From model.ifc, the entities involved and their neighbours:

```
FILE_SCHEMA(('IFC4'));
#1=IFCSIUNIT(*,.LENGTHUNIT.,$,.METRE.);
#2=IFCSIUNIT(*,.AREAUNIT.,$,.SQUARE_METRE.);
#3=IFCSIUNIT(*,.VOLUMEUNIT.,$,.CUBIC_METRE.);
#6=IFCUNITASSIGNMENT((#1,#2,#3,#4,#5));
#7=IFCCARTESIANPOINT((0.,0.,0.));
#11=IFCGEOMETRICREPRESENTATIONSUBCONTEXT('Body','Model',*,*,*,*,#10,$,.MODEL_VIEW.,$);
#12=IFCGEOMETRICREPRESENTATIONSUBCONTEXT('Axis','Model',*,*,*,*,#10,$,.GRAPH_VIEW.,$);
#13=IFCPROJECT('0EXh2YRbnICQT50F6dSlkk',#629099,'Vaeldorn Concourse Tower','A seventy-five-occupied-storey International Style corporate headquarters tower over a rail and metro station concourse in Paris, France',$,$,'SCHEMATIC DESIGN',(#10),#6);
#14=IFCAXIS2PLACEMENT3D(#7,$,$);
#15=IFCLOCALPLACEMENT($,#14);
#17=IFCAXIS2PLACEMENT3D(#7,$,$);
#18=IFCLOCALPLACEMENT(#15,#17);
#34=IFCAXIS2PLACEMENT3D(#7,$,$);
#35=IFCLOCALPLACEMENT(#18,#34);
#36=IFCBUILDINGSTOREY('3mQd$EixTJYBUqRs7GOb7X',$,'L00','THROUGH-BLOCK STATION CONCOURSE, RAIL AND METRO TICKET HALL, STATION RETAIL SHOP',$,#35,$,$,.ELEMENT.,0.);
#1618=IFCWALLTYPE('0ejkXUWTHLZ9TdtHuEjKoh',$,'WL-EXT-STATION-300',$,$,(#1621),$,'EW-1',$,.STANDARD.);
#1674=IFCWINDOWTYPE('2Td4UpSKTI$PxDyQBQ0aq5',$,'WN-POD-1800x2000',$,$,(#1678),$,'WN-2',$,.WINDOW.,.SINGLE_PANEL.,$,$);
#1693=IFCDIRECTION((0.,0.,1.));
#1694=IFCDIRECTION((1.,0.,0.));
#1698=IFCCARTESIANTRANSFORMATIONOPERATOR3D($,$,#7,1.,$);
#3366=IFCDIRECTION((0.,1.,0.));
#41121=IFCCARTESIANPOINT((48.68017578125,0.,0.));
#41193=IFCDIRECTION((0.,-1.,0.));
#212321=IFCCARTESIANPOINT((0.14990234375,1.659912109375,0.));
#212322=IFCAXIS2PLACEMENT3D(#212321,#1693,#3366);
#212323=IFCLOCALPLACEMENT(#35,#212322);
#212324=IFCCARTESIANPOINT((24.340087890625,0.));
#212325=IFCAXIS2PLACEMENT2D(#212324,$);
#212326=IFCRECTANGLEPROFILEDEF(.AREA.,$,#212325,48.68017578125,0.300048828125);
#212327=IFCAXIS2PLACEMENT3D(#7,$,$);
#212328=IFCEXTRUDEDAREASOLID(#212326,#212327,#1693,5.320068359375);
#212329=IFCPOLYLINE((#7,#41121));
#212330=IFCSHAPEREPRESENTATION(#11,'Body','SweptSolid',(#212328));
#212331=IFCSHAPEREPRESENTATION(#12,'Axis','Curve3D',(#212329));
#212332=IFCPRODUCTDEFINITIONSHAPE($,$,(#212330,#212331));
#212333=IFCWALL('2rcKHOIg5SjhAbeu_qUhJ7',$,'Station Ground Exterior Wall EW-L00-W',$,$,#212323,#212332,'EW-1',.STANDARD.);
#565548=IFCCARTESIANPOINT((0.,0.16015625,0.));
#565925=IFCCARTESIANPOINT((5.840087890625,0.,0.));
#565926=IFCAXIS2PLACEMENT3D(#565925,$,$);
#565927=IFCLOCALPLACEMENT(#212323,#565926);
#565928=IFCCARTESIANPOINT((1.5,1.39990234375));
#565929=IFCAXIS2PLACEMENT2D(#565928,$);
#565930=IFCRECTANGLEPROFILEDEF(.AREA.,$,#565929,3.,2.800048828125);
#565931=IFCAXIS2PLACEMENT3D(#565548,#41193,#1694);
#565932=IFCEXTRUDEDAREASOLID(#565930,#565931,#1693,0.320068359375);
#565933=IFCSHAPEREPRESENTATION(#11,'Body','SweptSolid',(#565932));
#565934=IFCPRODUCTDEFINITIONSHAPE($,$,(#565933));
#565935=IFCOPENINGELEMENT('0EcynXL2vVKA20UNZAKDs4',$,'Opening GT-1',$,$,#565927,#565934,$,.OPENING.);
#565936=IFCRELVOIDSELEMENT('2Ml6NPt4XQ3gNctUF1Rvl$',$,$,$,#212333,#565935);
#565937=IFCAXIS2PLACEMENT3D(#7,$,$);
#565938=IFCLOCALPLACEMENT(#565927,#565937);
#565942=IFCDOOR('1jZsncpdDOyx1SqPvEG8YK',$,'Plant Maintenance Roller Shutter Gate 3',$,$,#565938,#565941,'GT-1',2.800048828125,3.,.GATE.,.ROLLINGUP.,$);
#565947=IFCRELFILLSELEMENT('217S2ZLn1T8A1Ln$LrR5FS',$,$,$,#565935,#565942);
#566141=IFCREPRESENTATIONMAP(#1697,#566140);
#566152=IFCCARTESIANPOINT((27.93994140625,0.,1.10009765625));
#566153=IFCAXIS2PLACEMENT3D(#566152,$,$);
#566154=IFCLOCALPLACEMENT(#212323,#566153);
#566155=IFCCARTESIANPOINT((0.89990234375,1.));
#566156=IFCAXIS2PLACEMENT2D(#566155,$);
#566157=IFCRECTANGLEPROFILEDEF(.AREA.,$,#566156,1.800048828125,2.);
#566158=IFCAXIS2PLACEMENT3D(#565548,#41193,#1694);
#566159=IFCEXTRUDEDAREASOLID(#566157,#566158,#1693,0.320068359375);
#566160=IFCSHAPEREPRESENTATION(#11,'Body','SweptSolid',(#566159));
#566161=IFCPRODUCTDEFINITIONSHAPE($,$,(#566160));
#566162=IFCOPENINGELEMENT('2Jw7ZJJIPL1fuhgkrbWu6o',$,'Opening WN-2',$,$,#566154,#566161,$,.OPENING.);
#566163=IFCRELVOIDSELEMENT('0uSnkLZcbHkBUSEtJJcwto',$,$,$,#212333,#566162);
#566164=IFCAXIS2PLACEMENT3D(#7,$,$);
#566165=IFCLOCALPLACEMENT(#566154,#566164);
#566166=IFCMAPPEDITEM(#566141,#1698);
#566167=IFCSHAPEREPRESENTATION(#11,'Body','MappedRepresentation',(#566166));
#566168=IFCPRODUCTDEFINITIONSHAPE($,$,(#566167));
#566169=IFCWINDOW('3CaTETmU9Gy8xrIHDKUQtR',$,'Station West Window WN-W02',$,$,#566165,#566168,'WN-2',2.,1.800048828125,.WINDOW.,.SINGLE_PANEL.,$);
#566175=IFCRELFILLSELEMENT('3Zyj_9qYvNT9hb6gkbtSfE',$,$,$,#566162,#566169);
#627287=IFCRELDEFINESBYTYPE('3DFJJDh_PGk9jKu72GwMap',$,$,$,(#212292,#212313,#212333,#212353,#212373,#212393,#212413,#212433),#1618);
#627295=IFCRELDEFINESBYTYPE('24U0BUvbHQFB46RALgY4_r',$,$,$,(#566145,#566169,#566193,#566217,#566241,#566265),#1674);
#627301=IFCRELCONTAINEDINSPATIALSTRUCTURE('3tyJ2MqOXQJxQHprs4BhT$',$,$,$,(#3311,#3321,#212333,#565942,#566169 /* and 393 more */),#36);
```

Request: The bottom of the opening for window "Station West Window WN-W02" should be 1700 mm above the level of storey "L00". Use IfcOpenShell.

```python
import numpy as np
import ifcopenshell
import ifcopenshell.api.geometry
import ifcopenshell.geom
import ifcopenshell.util.element
import ifcopenshell.util.placement
import ifcopenshell.util.shape
import ifcopenshell.util.unit

model = ifcopenshell.open("model.ifc")
unit_scale = ifcopenshell.util.unit.calculate_unit_scale(model)

window = model.by_guid("3CaTETmU9Gy8xrIHDKUQtR")
opening = window.FillsVoids[0].RelatingOpeningElement
storey = ifcopenshell.util.element.get_container(window, ifc_class="IfcBuildingStorey")
level = ifcopenshell.util.placement.get_local_placement(storey.ObjectPlacement)[2, 3]

# The opening's origin need not be at the sill, so measure its lowest point.
shape = ifcopenshell.geom.create_shape(ifcopenshell.geom.settings(), opening)
bottom = ifcopenshell.util.shape.get_shape_bottom_elevation(shape, shape.geometry) / unit_scale
dz = level + 1.7 - bottom

shift = np.array([0.0, 0.0, dz])
# The window is placed relative to its opening, so it follows when the opening moves.
matrix = ifcopenshell.util.placement.get_local_placement(opening.ObjectPlacement)
matrix[:3, 3] += shift
ifcopenshell.api.geometry.edit_object_placement(
    model, product=opening, matrix=matrix, is_si=False, should_transform_children=True
)

print(f"moved by {dz * unit_scale:+.3f} m")

model.write("model-out.ifc")
```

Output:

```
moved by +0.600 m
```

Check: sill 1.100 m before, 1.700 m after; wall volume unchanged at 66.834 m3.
